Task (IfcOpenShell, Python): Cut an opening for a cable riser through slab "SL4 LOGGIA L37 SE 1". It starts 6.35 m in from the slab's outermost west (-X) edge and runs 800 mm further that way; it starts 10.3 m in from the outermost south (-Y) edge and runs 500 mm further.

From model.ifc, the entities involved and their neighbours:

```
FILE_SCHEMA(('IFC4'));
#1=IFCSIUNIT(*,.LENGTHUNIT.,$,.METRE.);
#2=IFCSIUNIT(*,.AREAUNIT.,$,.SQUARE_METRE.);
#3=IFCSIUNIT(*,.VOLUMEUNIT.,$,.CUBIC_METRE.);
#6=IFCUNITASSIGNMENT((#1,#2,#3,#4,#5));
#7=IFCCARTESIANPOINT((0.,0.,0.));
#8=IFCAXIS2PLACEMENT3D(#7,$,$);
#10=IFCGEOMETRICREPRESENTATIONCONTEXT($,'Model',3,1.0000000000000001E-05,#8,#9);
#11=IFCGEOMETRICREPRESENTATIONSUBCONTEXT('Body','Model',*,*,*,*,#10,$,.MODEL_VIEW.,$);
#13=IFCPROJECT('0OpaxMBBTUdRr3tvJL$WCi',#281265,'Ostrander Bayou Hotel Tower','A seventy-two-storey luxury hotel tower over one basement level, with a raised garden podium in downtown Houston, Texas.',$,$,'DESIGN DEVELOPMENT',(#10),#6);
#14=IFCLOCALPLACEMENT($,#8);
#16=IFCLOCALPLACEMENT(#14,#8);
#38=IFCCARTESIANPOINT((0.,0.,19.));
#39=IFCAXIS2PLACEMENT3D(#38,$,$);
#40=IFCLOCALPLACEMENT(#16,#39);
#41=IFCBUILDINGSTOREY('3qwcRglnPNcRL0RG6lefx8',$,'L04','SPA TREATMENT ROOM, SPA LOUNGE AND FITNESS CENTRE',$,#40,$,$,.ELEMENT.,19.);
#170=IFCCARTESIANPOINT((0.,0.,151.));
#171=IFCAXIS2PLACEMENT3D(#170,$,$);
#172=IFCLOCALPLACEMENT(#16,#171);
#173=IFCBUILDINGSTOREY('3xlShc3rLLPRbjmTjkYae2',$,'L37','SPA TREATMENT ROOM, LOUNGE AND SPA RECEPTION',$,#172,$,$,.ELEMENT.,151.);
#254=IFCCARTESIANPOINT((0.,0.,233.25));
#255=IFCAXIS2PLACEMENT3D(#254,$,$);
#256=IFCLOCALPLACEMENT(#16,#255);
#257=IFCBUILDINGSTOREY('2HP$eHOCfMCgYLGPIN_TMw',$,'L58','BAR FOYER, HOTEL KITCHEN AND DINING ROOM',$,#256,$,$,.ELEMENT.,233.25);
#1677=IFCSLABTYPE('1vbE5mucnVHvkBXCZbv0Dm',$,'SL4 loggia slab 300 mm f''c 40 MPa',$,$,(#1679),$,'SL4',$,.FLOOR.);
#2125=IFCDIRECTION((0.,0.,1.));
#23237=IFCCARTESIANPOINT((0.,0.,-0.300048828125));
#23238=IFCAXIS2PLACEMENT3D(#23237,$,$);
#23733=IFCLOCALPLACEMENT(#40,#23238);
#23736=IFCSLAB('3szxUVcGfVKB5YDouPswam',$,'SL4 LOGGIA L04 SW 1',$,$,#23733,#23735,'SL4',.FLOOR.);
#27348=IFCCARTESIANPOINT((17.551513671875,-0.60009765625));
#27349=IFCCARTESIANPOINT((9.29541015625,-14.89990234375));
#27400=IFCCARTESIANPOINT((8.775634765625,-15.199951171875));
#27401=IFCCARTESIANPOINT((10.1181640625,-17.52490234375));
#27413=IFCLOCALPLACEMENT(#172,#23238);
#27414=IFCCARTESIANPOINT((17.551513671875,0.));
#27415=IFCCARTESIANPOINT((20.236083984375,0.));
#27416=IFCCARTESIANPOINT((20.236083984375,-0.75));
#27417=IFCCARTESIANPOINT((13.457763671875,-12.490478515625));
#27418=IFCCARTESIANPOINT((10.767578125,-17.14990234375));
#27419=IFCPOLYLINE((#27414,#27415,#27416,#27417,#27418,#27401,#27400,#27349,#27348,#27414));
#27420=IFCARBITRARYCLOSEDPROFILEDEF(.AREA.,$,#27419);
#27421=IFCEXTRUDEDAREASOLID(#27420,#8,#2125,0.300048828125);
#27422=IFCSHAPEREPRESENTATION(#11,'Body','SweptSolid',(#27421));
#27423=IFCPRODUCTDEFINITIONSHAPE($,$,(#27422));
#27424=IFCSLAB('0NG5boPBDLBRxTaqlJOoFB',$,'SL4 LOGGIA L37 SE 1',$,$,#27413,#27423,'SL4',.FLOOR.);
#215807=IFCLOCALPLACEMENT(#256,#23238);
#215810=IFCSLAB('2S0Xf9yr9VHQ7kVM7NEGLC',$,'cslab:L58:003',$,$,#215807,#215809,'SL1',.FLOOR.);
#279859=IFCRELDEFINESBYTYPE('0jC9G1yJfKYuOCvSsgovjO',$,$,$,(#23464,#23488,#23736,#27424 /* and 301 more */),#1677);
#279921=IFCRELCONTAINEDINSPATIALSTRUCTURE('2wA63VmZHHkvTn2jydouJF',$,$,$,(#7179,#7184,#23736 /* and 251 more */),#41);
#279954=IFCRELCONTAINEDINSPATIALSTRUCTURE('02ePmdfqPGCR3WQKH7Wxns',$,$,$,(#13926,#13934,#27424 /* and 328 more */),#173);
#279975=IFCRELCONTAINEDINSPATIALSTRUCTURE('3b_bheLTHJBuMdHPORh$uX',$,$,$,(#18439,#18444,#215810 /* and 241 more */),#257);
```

```python
import numpy as np
import ifcopenshell
import ifcopenshell.api.feature
import ifcopenshell.api.geometry
import ifcopenshell.api.root
import ifcopenshell.geom
import ifcopenshell.util.placement
import ifcopenshell.util.representation
import ifcopenshell.util.shape
import ifcopenshell.util.unit

model = ifcopenshell.open("model.ifc")
unit_scale = ifcopenshell.util.unit.calculate_unit_scale(model)
settings = ifcopenshell.geom.settings()


def volume(element):
    """Net volume in cubic metres, openings subtracted."""
    shape = ifcopenshell.geom.create_shape(settings, element)
    return ifcopenshell.util.shape.get_volume(shape.geometry)


slab = model.by_guid("0NG5boPBDLBRxTaqlJOoFB")
before = volume(slab)

# Extent in the slab's own axes, in metres. The edges named are its -X and -Y sides.
slab_shape = ifcopenshell.geom.create_shape(settings, slab)
vertices = ifcopenshell.util.shape.get_vertices(slab_shape.geometry)
x_min, y_min, bottom = vertices.min(axis=0)
top = vertices[:, 2].max()

opening = ifcopenshell.api.root.create_entity(model, ifc_class="IfcOpeningElement", name="Cable riser opening", predefined_type="OPENING")
context = ifcopenshell.util.representation.get_context(model, "Model", "Body", "MODEL_VIEW")
width, depth = 0.8, 0.5
outline = [(0.0, 0.0), (width, 0.0), (width, depth), (0.0, depth), (0.0, 0.0)]
# Overshoot both faces by 50 mm so the cut is clean.
shape = ifcopenshell.api.geometry.add_slab_representation(
    model, context=context, depth=top - bottom + 0.1, polyline=outline
)
ifcopenshell.api.geometry.assign_representation(model, product=opening, representation=shape)

matrix = ifcopenshell.util.placement.get_local_placement(slab.ObjectPlacement)
matrix[:, 3] = matrix @ np.append(np.array([x_min + 6.35, y_min + 10.3, bottom - 0.05]) / unit_scale, 1.0)
ifcopenshell.api.geometry.edit_object_placement(model, product=opening, matrix=matrix, is_si=False)
ifcopenshell.api.feature.add_feature(model, feature=opening, element=slab)

after = volume(slab)

print(f"slab volume {before:.3f} -> {after:.3f} m3")

model.write("model-out.ifc")
```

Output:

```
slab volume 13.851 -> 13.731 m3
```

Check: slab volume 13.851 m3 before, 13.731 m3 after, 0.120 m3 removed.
